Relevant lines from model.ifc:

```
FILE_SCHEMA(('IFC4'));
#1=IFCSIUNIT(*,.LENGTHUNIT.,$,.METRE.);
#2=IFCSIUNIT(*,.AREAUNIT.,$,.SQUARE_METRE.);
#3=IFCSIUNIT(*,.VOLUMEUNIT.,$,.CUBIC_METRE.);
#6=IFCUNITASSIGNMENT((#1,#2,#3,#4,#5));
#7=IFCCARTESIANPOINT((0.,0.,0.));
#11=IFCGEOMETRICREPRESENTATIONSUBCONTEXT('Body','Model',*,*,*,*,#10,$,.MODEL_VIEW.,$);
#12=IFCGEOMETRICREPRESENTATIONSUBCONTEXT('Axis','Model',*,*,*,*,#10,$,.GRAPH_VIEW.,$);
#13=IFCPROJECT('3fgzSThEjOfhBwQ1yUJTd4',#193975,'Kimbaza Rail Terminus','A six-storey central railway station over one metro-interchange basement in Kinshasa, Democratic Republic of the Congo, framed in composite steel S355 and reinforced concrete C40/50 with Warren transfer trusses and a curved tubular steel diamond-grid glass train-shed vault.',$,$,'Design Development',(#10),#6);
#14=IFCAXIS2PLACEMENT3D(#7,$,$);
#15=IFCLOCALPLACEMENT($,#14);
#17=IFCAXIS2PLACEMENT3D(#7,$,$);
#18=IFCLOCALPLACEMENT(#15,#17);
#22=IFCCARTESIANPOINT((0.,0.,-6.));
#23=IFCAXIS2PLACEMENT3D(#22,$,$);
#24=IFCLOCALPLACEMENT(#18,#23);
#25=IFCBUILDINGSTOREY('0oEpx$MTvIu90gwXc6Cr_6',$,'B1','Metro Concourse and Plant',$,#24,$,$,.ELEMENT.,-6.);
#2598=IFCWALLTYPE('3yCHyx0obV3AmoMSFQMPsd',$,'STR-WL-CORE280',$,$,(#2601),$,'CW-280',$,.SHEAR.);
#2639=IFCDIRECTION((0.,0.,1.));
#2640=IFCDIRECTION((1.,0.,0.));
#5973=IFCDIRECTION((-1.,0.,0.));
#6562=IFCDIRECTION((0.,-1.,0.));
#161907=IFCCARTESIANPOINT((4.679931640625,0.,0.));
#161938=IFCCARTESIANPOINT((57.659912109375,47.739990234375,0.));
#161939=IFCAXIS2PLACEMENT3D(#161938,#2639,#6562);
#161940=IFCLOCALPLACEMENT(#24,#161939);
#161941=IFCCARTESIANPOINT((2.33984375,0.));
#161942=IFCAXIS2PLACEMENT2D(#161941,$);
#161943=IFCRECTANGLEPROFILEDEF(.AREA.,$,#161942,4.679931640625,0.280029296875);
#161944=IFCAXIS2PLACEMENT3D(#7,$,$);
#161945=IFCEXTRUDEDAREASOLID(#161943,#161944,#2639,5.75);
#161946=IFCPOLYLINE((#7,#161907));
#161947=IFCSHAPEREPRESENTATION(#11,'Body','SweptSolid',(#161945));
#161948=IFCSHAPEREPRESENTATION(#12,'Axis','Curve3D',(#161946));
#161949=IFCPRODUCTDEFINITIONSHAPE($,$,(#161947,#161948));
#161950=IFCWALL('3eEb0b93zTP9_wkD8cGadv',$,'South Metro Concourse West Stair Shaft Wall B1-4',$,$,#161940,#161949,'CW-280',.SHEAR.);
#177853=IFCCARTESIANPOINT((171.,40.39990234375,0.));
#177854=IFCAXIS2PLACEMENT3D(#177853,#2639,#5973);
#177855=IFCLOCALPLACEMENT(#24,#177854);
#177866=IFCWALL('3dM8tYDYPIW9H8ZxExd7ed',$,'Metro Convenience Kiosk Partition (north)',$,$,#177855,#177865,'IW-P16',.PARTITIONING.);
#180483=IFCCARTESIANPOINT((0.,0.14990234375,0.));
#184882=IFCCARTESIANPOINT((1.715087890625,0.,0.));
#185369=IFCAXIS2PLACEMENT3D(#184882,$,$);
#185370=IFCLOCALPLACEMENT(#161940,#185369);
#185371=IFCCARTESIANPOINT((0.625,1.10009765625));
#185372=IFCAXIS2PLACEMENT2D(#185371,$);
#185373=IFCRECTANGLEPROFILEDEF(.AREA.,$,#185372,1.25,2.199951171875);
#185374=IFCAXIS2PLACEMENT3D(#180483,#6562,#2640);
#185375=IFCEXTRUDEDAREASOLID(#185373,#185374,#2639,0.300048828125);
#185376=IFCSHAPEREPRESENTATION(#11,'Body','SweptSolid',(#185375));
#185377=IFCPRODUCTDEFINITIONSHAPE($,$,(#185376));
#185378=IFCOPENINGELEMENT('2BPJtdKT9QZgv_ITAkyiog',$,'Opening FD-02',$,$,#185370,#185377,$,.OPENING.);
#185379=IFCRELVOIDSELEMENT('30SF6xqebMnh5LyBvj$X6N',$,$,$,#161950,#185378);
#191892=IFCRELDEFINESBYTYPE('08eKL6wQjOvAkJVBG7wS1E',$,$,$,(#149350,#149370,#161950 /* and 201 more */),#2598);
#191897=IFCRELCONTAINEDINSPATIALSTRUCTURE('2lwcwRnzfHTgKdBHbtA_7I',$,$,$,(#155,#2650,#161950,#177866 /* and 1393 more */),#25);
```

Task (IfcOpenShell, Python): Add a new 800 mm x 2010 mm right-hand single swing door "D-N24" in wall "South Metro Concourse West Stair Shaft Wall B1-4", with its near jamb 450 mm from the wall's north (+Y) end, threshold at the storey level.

```python
import numpy as np
import ifcopenshell
import ifcopenshell.api.feature
import ifcopenshell.api.geometry
import ifcopenshell.api.root
import ifcopenshell.api.spatial
import ifcopenshell.geom
import ifcopenshell.util.element
import ifcopenshell.util.placement
import ifcopenshell.util.representation
import ifcopenshell.util.shape
import ifcopenshell.util.unit

model = ifcopenshell.open("model.ifc")
unit_scale = ifcopenshell.util.unit.calculate_unit_scale(model)
settings = ifcopenshell.geom.settings()


def volume(element):
    """Net volume in cubic metres, openings subtracted."""
    shape = ifcopenshell.geom.create_shape(settings, element)
    return ifcopenshell.util.shape.get_volume(shape.geometry)


wall = model.by_guid("3eEb0b93zTP9_wkD8cGadv")
storey = ifcopenshell.util.element.get_container(wall, ifc_class="IfcBuildingStorey")
context = ifcopenshell.util.representation.get_context(model, "Model", "Body", "MODEL_VIEW")
before = volume(wall)

width, height, from_end, sill = 0.8, 2.01, 0.45, 0.0  # metres

# The wall runs along its own X axis, and the end named is its -X end.
wall_shape = ifcopenshell.geom.create_shape(settings, wall)
x, y, z = ifcopenshell.util.shape.get_vertices(wall_shape.geometry).T
start = x.min() + from_end
face, thickness = float(y.min()), float(y.max() - y.min())
wall_matrix = ifcopenshell.util.placement.get_local_placement(wall.ObjectPlacement)
level = ifcopenshell.util.placement.get_local_placement(storey.ObjectPlacement)[2, 3]


def in_wall(x, y):
    """Placement at x, y metres in the wall's axes, at sill height."""
    matrix = wall_matrix.copy()
    matrix[:, 3] = wall_matrix @ np.array([x / unit_scale, y / unit_scale, 0.0, 1.0])
    matrix[2, 3] = level + sill / unit_scale
    return matrix


# Opening: a box that overshoots both wall faces by 50 mm.
opening = ifcopenshell.api.root.create_entity(model, ifc_class="IfcOpeningElement", predefined_type="OPENING")
box = ifcopenshell.api.geometry.add_wall_representation(
    model, context=context, length=width, height=height, thickness=thickness + 0.1
)
ifcopenshell.api.geometry.assign_representation(model, product=opening, representation=box)
ifcopenshell.api.geometry.edit_object_placement(model, product=opening, matrix=in_wall(start, face - 0.05), is_si=False)
ifcopenshell.api.feature.add_feature(model, feature=opening, element=wall)

door = ifcopenshell.api.root.create_entity(model, ifc_class="IfcDoor", name="D-N24", predefined_type="DOOR")
door.OverallWidth, door.OverallHeight = width / unit_scale, height / unit_scale
door.OperationType = "SINGLE_SWING_RIGHT"
body = ifcopenshell.api.geometry.add_door_representation(
    model,
    context=context,
    overall_width=door.OverallWidth,
    overall_height=door.OverallHeight,
    operation_type="SINGLE_SWING_RIGHT",
    lining_properties={"LiningDepth": thickness / unit_scale, "ThresholdDepth": thickness / unit_scale},
)
ifcopenshell.api.geometry.assign_representation(model, product=door, representation=body)
ifcopenshell.api.spatial.assign_container(model, products=[door], relating_structure=storey)
ifcopenshell.api.feature.add_filling(model, opening=opening, element=door)

# The lining spans the wall, so the door starts at the wall face.
ifcopenshell.api.geometry.edit_object_placement(model, product=door, matrix=in_wall(start, face), is_si=False)

after = volume(wall)

print(f"wall volume {before:.3f} -> {after:.3f} m3")

model.write("model_edited.ifc")
```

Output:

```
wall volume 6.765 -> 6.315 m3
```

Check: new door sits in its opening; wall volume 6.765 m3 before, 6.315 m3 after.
